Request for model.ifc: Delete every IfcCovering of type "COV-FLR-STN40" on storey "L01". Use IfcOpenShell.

First a look at what the model holds.

```python
import ifcopenshell
import ifcopenshell.util.element

model = ifcopenshell.open("model.ifc")
print(model.schema)
storey = next(s for s in model.by_type("IfcBuildingStorey") if s.Name == "L01")
coverings = [e for e in ifcopenshell.util.element.get_decomposition(storey) if e.is_a("IfcCovering")]
seen = {}
for e in coverings:
    element_type = ifcopenshell.util.element.get_type(e)
    name = element_type.Name if element_type not in (None, e) else None
    seen[name] = seen.get(name, 0) + 1
for name, count in sorted(seen.items(), key=str):
    print(count, "x", name)
```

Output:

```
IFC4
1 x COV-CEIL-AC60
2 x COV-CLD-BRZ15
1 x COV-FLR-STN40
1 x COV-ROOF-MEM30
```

```python
import ifcopenshell
import ifcopenshell.api.root
import ifcopenshell.util.element

model = ifcopenshell.open("model.ifc")

storey = next(s for s in model.by_type("IfcBuildingStorey") if s.Name == "L01")
coverings = [e for e in ifcopenshell.util.element.get_decomposition(storey) if e.is_a("IfcCovering")]
targets = [e for e in coverings if (t := ifcopenshell.util.element.get_type(e)) not in (None, e) and t.Name == "COV-FLR-STN40"]

for e in targets:
    ifcopenshell.api.root.remove_product(model, product=e)
print(len(targets), "removed")

model.write("model_v2.ifc")
```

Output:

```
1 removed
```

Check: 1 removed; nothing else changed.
